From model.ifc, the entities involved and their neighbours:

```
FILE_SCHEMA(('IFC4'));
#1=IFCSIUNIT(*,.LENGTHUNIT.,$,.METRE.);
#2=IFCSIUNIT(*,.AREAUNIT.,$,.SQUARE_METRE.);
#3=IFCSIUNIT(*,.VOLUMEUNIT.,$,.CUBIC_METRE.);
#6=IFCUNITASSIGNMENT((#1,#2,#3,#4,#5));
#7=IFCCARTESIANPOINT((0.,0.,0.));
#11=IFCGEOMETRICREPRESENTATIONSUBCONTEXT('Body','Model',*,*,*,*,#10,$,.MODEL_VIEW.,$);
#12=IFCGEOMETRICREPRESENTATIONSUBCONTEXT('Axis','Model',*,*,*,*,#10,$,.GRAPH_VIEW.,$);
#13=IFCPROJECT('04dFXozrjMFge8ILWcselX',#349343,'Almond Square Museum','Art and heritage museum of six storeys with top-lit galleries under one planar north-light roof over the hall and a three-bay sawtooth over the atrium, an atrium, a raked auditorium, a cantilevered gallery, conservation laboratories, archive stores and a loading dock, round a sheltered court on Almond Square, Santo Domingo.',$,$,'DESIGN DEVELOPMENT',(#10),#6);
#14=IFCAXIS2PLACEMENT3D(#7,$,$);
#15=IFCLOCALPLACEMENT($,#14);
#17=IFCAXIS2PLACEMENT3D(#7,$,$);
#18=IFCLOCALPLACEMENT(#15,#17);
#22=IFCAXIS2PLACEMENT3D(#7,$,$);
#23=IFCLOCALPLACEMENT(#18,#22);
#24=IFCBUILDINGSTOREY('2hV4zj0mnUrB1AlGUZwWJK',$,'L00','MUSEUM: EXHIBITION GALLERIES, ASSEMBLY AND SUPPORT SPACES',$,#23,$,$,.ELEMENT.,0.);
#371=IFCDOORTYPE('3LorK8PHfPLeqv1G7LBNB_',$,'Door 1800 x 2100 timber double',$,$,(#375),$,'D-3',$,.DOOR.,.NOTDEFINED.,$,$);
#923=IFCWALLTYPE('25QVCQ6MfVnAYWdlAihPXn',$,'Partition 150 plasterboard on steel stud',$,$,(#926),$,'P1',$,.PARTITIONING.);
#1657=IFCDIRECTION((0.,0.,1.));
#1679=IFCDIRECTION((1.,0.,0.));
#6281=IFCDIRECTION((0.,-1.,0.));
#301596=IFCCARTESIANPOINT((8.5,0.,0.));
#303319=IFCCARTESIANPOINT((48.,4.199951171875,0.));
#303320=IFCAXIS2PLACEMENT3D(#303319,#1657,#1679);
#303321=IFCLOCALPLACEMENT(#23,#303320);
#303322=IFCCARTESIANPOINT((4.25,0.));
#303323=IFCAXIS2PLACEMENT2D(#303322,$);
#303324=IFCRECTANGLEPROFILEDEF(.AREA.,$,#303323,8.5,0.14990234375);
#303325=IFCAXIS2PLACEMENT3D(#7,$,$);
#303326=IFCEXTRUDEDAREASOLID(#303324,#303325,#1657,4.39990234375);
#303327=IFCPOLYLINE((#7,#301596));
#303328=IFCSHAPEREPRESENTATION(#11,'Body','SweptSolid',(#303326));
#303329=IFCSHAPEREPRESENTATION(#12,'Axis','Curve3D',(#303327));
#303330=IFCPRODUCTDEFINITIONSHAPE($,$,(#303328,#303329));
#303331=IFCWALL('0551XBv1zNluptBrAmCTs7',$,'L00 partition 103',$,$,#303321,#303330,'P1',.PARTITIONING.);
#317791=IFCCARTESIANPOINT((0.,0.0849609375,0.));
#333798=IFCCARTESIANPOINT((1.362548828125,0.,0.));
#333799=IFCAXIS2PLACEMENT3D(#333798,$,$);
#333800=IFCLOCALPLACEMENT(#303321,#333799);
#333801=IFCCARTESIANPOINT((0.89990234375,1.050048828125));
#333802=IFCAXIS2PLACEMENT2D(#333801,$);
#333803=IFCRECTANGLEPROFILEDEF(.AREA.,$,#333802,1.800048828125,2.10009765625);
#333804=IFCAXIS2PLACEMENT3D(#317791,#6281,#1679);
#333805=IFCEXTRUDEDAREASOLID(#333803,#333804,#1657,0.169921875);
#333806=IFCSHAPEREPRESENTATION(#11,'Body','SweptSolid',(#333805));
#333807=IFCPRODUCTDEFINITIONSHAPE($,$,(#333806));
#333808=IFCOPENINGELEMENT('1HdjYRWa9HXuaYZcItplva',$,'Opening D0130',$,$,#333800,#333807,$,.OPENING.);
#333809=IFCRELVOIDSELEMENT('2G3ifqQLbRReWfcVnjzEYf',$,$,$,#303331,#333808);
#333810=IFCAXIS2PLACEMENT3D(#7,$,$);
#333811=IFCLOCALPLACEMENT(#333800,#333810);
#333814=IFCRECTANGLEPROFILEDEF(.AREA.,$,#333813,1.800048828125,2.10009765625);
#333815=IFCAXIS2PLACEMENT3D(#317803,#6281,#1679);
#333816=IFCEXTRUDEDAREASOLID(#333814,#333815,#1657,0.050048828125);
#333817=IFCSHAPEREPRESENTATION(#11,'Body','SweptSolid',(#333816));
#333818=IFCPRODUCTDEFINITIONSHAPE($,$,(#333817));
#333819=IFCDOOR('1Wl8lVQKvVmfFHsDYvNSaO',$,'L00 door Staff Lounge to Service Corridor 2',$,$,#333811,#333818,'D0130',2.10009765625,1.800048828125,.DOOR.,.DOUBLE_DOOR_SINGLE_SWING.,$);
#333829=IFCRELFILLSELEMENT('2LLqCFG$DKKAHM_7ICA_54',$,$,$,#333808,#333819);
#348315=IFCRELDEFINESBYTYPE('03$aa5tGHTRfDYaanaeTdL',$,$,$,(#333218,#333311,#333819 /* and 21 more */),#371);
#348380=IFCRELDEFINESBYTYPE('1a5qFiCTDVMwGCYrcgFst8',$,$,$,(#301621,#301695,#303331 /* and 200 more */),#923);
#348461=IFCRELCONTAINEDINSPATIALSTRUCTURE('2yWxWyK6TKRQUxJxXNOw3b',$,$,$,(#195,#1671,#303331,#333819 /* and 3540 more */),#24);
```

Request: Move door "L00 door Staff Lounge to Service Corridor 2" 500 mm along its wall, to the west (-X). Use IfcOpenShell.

```python
import ifcopenshell
import ifcopenshell.api.geometry
import ifcopenshell.util.placement

model = ifcopenshell.open("model.ifc")

door = model.by_id(333819)
opening = door.FillsVoids[0].RelatingOpeningElement
wall = opening.VoidsElements[0].RelatingBuildingElement

wall_matrix = ifcopenshell.util.placement.get_local_placement(wall.ObjectPlacement)
shift = wall_matrix[:3, 0] * -0.5
before = ifcopenshell.util.placement.get_local_placement(door.ObjectPlacement)[:3, 3].copy()

# The door is placed relative to its opening, so it follows when the opening moves.
matrix = ifcopenshell.util.placement.get_local_placement(opening.ObjectPlacement)
matrix[:3, 3] += shift
ifcopenshell.api.geometry.edit_object_placement(
    model, product=opening, matrix=matrix, is_si=False, should_transform_children=True
)

after = ifcopenshell.util.placement.get_local_placement(door.ObjectPlacement)[:3, 3]
print("door moved by", (after - before).round(3) + 0.0)

model.write("model_updated.ifc")
```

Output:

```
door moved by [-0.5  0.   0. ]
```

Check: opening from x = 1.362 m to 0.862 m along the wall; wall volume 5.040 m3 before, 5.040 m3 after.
